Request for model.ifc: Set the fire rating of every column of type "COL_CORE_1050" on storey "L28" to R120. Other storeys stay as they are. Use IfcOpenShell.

First a look at what the model holds.

```python
import ifcopenshell
import ifcopenshell.util.element

model = ifcopenshell.open("model.ifc")
print(model.schema)
storey = next(s for s in model.by_type("IfcBuildingStorey") if s.Name == "L28")
columns = [e for e in ifcopenshell.util.element.get_decomposition(storey) if e.is_a("IfcColumn")]
seen = {}
for e in columns:
    element_type = ifcopenshell.util.element.get_type(e)
    key = (element_type.Name if element_type != e and element_type else None, ifcopenshell.util.element.get_pset(e, "Pset_ColumnCommon", "FireRating"))
    seen[key] = seen.get(key, 0) + 1
for (name, value), count in sorted(seen.items(), key=str):
    print(count, "x", name, "|", value)
```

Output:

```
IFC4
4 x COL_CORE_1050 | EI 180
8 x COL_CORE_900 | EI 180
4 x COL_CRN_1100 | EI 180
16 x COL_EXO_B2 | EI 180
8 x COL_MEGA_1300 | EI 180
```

```python
import ifcopenshell
import ifcopenshell.api.pset
import ifcopenshell.util.element

model = ifcopenshell.open("model.ifc")

storey = next(s for s in model.by_type("IfcBuildingStorey") if s.Name == "L28")
columns = [e for e in ifcopenshell.util.element.get_decomposition(storey) if e.is_a("IfcColumn")]

count = 0
for e in columns:
    element_type = ifcopenshell.util.element.get_type(e)
    if element_type in (None, e) or element_type.Name != "COL_CORE_1050":
        continue
    found = ifcopenshell.util.element.get_pset(e, "Pset_ColumnCommon", should_inherit=False)
    if found:
        pset = model.by_id(found["id"])
        if len(ifcopenshell.util.element.get_elements_by_pset(pset)) > 1:
            pset = ifcopenshell.api.pset.unshare_pset(model, products=[e], pset=pset)[0]
    else:
        pset = ifcopenshell.api.pset.add_pset(model, product=e, name="Pset_ColumnCommon")
    ifcopenshell.api.pset.edit_pset(model, pset=pset, properties={"FireRating": "R120"})
    count += 1

print(count, "columns updated")

model.write("model_rev.ifc")
```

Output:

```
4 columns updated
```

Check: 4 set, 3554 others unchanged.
